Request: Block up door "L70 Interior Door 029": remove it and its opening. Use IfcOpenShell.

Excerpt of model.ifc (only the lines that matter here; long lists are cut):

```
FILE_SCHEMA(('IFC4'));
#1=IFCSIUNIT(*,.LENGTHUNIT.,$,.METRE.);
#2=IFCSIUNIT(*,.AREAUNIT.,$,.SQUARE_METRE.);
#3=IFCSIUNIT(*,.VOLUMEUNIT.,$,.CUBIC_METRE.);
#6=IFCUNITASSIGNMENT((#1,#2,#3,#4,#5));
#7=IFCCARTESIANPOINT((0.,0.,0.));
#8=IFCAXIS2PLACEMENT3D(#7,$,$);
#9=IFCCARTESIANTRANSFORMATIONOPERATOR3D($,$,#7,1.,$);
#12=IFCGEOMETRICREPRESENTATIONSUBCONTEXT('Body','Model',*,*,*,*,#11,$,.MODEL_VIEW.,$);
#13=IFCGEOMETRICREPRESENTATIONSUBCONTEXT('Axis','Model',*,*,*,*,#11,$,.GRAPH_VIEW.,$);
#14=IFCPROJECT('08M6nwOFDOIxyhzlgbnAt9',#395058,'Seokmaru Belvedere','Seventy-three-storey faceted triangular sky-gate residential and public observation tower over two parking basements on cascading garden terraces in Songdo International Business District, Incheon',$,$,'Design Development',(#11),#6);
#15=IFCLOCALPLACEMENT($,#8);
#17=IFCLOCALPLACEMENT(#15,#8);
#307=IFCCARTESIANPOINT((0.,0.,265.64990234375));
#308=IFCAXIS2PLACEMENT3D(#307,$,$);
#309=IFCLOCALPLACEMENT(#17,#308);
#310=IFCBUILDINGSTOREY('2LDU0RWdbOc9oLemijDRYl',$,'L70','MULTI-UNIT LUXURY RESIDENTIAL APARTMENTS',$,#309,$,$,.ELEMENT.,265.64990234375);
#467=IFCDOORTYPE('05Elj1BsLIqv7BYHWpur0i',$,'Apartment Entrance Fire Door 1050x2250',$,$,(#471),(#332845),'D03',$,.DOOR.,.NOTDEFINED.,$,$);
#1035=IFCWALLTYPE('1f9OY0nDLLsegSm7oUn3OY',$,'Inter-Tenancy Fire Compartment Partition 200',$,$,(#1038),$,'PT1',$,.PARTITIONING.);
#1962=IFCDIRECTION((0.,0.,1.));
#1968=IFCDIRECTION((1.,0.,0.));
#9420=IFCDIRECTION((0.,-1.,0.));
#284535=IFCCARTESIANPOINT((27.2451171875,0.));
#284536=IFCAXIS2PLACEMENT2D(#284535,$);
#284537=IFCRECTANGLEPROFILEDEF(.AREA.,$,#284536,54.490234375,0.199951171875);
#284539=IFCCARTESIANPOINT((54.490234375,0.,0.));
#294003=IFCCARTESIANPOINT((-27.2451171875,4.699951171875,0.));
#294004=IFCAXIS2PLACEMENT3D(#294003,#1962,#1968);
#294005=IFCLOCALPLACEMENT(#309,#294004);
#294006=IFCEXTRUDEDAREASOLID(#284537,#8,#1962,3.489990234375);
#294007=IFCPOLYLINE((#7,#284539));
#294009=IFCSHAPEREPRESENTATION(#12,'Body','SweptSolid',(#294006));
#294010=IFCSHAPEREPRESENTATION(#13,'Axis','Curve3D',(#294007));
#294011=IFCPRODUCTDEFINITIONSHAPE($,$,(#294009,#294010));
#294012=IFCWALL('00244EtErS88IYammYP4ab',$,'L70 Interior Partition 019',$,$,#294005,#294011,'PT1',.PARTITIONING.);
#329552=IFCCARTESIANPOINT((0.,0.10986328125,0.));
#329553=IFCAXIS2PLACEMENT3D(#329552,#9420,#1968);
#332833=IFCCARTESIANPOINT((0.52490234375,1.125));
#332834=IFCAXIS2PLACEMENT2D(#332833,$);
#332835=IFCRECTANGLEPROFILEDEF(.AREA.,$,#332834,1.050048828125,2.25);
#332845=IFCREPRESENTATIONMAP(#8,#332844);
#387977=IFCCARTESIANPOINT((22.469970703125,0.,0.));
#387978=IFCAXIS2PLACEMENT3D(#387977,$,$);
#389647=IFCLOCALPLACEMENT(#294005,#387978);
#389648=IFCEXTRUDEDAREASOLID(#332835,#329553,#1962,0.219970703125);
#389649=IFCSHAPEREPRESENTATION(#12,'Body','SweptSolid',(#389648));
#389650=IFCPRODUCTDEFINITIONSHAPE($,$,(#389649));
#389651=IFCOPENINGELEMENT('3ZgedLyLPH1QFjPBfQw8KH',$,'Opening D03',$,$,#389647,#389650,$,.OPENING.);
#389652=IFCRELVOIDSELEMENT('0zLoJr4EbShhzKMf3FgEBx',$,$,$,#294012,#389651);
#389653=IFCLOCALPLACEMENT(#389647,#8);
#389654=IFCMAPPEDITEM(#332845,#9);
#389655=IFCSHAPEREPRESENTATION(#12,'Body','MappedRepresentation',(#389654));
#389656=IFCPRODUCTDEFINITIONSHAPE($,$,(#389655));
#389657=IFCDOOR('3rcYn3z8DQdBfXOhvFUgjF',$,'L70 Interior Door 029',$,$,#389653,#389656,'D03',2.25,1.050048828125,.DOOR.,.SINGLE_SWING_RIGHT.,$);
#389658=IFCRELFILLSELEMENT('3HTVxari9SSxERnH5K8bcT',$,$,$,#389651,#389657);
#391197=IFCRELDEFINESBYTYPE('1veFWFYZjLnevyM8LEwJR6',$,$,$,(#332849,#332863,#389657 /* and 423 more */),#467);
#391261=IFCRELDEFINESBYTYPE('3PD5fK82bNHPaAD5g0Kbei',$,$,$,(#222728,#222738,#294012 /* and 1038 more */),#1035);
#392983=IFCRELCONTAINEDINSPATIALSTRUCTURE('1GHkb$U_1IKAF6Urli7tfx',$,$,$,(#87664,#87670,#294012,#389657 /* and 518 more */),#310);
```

```python
import ifcopenshell
import ifcopenshell.api.feature
import ifcopenshell.api.root
import ifcopenshell.geom
import ifcopenshell.util.shape

model = ifcopenshell.open("model.ifc")
settings = ifcopenshell.geom.settings()


def volume(element):
    """Net volume in cubic metres, openings subtracted."""
    shape = ifcopenshell.geom.create_shape(settings, element)
    return ifcopenshell.util.shape.get_volume(shape.geometry)


door = model.by_guid("3rcYn3z8DQdBfXOhvFUgjF")
opening = door.FillsVoids[0].RelatingOpeningElement
wall = opening.VoidsElements[0].RelatingBuildingElement
before = volume(wall)

ifcopenshell.api.root.remove_product(model, product=door)
ifcopenshell.api.feature.remove_feature(model, feature=opening)

after = volume(wall)

print(f"wall volume {before:.3f} -> {after:.3f} m3")

model.write("model_edited.ifc")
```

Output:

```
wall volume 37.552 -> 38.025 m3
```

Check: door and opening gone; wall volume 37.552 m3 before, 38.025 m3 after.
